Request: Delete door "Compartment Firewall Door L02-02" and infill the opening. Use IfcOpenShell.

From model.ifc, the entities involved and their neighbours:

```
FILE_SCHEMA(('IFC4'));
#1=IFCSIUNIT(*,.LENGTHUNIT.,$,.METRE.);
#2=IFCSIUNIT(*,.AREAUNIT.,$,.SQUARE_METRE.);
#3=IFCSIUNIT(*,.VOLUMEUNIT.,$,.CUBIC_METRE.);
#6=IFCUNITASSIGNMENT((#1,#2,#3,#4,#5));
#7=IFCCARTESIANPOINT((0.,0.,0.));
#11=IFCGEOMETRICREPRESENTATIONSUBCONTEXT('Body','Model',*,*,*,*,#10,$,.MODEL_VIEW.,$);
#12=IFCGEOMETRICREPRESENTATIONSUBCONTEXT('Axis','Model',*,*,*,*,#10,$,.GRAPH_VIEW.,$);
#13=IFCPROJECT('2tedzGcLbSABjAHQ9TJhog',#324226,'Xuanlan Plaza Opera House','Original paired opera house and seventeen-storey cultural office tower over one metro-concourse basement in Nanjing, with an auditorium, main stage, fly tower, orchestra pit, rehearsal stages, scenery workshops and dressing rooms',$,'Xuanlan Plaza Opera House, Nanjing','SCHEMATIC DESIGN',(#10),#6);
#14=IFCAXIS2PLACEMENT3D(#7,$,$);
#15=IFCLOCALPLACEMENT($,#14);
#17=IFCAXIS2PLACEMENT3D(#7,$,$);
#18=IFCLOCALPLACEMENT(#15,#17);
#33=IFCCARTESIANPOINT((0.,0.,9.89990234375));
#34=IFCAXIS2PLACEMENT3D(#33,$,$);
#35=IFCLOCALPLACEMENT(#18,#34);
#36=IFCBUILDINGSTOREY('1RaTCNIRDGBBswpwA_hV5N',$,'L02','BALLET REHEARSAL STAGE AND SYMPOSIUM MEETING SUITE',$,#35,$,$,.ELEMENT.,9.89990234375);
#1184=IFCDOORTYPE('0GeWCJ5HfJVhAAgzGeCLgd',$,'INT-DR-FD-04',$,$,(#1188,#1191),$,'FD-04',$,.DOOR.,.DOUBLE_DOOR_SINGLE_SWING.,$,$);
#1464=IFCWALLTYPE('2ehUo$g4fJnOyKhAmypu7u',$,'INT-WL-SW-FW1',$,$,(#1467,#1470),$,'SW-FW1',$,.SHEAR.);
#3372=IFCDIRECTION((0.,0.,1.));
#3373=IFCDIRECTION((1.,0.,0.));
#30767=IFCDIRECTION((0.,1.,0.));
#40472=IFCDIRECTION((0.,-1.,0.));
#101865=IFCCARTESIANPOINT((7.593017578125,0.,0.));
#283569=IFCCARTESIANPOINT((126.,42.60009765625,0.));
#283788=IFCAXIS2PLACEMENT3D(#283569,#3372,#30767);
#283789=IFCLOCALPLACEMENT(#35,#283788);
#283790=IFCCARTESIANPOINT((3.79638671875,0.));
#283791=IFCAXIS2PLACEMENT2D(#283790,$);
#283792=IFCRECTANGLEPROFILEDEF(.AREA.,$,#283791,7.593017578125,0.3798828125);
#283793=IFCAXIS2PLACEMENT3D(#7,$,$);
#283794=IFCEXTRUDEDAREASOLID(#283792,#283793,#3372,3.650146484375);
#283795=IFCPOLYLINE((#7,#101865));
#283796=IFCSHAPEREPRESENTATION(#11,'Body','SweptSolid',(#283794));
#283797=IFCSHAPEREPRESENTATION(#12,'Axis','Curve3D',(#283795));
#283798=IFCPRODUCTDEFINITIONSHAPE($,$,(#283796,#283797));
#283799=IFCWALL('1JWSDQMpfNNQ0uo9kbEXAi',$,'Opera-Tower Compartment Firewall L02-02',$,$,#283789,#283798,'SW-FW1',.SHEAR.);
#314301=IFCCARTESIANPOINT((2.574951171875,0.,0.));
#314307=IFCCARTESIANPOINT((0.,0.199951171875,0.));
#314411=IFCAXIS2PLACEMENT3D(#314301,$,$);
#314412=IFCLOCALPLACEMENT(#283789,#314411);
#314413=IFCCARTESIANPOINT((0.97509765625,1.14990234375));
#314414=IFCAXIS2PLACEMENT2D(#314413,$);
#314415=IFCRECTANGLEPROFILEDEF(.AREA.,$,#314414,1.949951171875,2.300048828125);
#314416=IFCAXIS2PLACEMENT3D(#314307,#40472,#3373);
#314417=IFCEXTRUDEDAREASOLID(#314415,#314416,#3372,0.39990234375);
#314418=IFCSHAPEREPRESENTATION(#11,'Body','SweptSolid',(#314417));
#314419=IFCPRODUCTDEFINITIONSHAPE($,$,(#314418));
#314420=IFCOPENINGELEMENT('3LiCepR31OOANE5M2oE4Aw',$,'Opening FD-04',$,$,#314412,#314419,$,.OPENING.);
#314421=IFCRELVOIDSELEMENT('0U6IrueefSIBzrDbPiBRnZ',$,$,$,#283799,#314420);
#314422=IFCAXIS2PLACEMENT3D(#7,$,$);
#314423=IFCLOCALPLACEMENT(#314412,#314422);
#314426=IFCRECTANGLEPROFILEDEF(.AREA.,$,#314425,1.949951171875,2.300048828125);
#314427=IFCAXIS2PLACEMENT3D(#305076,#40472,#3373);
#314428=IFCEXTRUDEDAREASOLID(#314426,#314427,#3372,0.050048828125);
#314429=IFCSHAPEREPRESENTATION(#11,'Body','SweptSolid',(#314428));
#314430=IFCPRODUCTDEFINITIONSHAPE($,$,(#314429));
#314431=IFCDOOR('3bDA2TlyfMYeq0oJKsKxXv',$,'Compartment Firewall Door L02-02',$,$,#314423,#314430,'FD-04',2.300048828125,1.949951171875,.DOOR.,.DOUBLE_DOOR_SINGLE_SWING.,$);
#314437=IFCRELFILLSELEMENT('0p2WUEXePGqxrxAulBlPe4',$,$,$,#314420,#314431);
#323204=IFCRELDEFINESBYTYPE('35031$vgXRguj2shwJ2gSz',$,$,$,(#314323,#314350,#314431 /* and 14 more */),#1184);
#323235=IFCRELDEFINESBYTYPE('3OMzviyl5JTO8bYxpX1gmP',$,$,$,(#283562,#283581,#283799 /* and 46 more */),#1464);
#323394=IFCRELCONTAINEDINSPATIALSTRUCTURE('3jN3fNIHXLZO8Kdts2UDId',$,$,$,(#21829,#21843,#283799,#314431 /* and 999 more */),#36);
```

```python
import ifcopenshell
import ifcopenshell.api.feature
import ifcopenshell.api.root
import ifcopenshell.geom
import ifcopenshell.util.shape

model = ifcopenshell.open("model.ifc")
settings = ifcopenshell.geom.settings()


def volume(element):
    """Net volume in cubic metres, openings subtracted."""
    shape = ifcopenshell.geom.create_shape(settings, element)
    return ifcopenshell.util.shape.get_volume(shape.geometry)


door = model.by_id(314431)
opening = door.FillsVoids[0].RelatingOpeningElement
wall = opening.VoidsElements[0].RelatingBuildingElement
before = volume(wall)

ifcopenshell.api.root.remove_product(model, product=door)
ifcopenshell.api.feature.remove_feature(model, feature=opening)

after = volume(wall)

print(f"wall volume {before:.3f} -> {after:.3f} m3")

model.write("model_edited.ifc")
```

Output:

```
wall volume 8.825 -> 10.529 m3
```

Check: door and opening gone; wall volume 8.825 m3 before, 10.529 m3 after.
